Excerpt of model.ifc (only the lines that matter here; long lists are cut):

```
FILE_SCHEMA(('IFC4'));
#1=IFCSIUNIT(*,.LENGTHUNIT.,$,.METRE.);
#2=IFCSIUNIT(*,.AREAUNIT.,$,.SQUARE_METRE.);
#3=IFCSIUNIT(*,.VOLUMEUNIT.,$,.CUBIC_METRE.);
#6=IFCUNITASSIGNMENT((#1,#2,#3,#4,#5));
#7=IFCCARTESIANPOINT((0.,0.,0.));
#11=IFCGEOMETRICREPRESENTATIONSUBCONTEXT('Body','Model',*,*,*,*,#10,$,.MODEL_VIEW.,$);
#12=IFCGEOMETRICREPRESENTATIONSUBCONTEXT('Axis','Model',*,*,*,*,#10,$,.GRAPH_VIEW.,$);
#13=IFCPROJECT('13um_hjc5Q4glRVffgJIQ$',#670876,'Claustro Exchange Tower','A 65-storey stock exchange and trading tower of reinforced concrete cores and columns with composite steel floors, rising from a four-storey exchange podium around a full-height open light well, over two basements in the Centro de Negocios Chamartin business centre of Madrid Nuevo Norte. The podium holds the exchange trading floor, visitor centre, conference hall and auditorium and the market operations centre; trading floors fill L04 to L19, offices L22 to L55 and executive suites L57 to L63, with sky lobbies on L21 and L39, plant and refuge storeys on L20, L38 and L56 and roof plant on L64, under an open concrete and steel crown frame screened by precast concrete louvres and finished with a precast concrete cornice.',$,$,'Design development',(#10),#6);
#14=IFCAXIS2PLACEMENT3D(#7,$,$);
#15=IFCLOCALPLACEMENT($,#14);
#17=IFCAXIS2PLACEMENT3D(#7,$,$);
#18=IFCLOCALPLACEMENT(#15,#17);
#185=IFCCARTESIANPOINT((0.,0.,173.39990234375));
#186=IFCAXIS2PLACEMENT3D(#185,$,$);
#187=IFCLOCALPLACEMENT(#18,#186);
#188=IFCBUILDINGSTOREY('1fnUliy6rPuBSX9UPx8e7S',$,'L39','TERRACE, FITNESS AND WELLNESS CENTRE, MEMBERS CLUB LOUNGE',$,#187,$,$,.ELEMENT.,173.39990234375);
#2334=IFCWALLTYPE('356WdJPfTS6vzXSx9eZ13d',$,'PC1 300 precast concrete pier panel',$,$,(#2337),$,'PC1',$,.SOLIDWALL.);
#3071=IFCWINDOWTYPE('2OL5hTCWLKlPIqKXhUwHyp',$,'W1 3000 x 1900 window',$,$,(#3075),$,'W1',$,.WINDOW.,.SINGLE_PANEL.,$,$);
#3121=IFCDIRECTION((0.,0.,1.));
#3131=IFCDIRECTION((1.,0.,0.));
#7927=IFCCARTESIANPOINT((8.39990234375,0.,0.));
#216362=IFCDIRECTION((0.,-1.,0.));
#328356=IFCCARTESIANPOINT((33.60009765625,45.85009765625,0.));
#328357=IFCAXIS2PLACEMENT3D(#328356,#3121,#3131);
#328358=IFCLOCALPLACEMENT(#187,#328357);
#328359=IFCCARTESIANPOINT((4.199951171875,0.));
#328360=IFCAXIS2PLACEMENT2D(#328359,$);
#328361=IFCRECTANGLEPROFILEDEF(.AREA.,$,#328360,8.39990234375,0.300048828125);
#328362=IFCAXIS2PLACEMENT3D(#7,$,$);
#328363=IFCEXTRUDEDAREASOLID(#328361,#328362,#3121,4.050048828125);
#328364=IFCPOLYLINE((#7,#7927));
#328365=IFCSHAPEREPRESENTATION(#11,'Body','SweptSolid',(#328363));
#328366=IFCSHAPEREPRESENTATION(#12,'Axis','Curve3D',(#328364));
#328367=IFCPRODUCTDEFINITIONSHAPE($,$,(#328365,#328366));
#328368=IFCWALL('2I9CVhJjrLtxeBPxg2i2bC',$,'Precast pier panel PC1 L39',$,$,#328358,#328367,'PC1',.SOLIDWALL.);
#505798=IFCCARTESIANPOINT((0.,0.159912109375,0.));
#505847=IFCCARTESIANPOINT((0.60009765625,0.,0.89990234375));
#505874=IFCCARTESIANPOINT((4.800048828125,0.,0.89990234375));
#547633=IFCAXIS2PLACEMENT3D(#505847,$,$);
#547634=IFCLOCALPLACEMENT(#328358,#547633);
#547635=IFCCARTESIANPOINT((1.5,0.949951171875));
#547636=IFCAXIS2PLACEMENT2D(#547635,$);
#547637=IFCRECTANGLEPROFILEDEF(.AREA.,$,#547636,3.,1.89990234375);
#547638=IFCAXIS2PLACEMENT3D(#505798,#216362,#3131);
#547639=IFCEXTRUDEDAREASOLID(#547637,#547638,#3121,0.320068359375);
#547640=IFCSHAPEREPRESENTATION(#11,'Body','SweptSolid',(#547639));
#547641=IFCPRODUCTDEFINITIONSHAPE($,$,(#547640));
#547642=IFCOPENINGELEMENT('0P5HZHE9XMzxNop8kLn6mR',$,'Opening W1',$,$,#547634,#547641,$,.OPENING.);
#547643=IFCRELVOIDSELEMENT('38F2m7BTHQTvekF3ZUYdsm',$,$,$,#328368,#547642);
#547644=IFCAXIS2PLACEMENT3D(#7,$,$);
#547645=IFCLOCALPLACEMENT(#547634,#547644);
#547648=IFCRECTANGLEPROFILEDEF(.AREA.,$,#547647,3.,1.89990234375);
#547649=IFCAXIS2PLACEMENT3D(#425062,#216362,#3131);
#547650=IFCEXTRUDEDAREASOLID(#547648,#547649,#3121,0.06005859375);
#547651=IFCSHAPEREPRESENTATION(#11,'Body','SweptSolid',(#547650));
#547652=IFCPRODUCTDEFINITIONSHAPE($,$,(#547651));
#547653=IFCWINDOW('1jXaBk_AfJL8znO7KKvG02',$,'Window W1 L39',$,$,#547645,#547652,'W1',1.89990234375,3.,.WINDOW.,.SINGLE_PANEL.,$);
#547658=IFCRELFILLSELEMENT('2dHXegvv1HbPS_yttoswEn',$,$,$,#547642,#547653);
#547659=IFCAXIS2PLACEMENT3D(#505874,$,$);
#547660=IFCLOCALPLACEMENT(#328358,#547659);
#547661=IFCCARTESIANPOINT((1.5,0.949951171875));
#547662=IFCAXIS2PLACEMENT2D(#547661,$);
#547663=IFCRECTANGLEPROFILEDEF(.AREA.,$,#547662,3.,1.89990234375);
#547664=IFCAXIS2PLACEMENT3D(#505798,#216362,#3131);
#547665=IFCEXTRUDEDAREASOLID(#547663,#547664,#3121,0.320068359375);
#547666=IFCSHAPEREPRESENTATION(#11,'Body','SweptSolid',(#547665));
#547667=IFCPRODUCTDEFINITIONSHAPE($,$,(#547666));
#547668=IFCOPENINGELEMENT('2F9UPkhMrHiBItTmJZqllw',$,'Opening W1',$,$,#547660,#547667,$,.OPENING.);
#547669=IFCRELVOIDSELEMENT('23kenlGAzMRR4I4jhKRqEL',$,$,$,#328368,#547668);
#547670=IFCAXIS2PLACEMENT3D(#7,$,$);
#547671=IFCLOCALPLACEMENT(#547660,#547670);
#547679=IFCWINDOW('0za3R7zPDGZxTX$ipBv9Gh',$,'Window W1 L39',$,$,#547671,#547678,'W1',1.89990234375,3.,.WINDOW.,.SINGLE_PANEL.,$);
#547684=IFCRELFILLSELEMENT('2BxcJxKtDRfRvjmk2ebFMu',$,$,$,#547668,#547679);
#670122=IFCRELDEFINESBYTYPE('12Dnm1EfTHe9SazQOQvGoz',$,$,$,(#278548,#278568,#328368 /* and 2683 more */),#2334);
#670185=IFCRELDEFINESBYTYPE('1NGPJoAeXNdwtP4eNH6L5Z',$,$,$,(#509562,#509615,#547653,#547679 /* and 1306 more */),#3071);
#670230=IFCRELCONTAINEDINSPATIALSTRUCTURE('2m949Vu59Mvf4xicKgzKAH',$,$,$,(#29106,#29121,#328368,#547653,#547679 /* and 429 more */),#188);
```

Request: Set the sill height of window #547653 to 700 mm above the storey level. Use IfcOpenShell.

```python
import numpy as np
import ifcopenshell
import ifcopenshell.api.geometry
import ifcopenshell.geom
import ifcopenshell.util.element
import ifcopenshell.util.placement
import ifcopenshell.util.shape
import ifcopenshell.util.unit

model = ifcopenshell.open("model.ifc")
unit_scale = ifcopenshell.util.unit.calculate_unit_scale(model)

window = model.by_guid("1jXaBk_AfJL8znO7KKvG02")
opening = window.FillsVoids[0].RelatingOpeningElement
storey = ifcopenshell.util.element.get_container(window, ifc_class="IfcBuildingStorey")
level = ifcopenshell.util.placement.get_local_placement(storey.ObjectPlacement)[2, 3]

# The opening's origin need not be at the sill, so measure its lowest point.
shape = ifcopenshell.geom.create_shape(ifcopenshell.geom.settings(), opening)
bottom = ifcopenshell.util.shape.get_shape_bottom_elevation(shape, shape.geometry) / unit_scale
dz = level + 0.7 - bottom

shift = np.array([0.0, 0.0, dz])
# The window is placed relative to its opening, so it follows when the opening moves.
matrix = ifcopenshell.util.placement.get_local_placement(opening.ObjectPlacement)
matrix[:3, 3] += shift
ifcopenshell.api.geometry.edit_object_placement(
    model, product=opening, matrix=matrix, is_si=False, should_transform_children=True
)

print(f"moved by {dz * unit_scale:+.3f} m")

model.write("model_updated.ifc")
```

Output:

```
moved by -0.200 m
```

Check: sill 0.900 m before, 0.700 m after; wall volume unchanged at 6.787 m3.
